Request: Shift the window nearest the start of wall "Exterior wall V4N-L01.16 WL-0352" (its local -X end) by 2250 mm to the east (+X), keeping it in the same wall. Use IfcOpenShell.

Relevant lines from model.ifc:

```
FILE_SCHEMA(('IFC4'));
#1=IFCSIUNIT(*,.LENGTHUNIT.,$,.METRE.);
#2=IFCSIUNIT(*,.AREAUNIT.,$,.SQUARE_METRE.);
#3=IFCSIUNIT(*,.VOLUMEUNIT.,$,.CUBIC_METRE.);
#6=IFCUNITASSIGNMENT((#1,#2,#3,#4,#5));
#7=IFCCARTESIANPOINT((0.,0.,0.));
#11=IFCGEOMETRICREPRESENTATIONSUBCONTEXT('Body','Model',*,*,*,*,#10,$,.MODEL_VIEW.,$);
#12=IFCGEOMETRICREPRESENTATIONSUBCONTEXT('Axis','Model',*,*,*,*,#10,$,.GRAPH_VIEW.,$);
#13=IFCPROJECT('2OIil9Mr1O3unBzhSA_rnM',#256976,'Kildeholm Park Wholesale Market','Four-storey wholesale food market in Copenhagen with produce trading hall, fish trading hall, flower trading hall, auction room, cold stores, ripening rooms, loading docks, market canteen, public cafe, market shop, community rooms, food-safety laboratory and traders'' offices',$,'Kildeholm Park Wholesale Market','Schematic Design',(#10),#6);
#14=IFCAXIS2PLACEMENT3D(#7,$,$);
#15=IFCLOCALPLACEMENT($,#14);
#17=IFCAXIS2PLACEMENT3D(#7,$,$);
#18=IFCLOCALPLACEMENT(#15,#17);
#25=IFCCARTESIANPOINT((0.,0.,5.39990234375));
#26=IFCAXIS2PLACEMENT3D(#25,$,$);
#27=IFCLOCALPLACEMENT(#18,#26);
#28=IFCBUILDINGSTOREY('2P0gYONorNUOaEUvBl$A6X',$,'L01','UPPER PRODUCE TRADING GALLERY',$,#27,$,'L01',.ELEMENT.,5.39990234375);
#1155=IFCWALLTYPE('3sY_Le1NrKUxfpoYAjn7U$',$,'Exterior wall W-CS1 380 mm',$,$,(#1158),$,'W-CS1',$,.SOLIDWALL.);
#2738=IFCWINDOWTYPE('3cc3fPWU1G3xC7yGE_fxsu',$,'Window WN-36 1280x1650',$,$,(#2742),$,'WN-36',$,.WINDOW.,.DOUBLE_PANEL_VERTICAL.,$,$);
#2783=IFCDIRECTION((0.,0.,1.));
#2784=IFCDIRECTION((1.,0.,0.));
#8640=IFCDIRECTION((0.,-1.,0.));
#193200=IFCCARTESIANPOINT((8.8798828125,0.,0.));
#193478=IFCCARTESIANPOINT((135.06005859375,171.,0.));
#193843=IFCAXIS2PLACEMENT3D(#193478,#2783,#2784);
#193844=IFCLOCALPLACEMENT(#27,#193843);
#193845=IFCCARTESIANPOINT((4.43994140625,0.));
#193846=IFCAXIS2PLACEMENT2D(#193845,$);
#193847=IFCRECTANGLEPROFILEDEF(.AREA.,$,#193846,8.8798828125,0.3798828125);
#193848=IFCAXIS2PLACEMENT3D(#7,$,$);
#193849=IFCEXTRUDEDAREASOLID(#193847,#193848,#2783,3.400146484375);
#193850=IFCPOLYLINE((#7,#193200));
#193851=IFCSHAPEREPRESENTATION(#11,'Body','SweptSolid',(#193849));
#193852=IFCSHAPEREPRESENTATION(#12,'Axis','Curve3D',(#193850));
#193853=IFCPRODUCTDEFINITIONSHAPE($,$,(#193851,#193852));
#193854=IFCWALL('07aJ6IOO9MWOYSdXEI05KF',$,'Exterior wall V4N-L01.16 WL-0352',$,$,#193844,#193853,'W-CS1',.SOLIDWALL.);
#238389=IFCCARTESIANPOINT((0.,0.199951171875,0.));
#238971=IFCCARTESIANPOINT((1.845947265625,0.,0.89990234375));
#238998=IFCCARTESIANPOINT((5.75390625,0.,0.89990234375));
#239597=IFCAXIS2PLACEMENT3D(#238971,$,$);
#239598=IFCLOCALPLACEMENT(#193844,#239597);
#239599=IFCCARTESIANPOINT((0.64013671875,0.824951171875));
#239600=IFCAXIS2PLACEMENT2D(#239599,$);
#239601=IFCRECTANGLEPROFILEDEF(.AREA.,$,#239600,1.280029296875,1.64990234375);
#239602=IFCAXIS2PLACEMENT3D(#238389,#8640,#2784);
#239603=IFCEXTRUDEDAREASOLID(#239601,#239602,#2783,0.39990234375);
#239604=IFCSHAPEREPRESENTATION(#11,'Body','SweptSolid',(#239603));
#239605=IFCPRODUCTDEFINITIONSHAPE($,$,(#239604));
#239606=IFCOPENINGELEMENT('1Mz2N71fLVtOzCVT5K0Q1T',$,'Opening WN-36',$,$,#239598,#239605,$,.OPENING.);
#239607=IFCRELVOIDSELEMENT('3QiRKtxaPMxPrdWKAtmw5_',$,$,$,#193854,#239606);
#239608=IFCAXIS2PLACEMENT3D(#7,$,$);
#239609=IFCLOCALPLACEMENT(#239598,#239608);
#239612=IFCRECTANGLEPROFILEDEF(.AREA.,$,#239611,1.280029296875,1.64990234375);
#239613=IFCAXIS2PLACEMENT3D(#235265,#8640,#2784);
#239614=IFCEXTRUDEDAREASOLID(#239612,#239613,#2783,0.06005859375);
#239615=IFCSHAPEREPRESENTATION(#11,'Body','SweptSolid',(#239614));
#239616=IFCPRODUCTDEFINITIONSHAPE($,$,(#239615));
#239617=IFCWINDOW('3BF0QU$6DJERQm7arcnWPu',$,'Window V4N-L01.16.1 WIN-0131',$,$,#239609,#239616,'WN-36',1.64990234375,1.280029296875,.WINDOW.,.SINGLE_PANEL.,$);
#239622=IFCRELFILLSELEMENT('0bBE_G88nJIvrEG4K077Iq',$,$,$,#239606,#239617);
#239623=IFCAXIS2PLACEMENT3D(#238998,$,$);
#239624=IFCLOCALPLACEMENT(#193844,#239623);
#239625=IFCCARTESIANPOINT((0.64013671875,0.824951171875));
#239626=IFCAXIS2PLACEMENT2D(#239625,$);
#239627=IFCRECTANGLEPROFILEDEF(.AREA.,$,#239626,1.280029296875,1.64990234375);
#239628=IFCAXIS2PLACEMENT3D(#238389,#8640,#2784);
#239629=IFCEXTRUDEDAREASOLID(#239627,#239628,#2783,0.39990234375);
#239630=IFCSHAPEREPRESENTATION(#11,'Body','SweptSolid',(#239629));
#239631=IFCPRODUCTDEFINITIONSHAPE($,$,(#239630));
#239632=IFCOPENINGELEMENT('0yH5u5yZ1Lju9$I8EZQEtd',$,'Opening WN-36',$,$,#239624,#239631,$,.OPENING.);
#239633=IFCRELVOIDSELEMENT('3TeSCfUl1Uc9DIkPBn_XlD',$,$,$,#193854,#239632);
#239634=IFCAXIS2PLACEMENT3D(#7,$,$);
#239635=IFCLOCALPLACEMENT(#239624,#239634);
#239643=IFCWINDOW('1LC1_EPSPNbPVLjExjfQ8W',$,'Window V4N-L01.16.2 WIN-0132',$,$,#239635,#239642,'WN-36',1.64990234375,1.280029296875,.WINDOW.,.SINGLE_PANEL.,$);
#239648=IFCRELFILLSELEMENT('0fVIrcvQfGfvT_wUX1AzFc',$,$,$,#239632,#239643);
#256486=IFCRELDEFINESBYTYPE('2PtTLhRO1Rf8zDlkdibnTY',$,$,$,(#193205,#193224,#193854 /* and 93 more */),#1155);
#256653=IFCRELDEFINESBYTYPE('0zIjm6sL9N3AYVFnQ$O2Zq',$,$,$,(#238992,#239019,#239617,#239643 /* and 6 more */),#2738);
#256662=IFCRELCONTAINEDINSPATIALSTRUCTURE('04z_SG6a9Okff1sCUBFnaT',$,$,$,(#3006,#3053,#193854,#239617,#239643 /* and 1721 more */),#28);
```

```python
import ifcopenshell
import ifcopenshell.api.geometry
import ifcopenshell.util.placement

model = ifcopenshell.open("model.ifc")

window = model.by_id(239617)
opening = window.FillsVoids[0].RelatingOpeningElement
wall = opening.VoidsElements[0].RelatingBuildingElement

wall_matrix = ifcopenshell.util.placement.get_local_placement(wall.ObjectPlacement)
shift = wall_matrix[:3, 0] * 2.25
before = ifcopenshell.util.placement.get_local_placement(window.ObjectPlacement)[:3, 3].copy()

# The window is placed relative to its opening, so it follows when the opening moves.
matrix = ifcopenshell.util.placement.get_local_placement(opening.ObjectPlacement)
matrix[:3, 3] += shift
ifcopenshell.api.geometry.edit_object_placement(
    model, product=opening, matrix=matrix, is_si=False, should_transform_children=True
)

after = ifcopenshell.util.placement.get_local_placement(window.ObjectPlacement)[:3, 3]
print("window moved by", (after - before).round(3) + 0.0)

model.write("model_updated.ifc")
```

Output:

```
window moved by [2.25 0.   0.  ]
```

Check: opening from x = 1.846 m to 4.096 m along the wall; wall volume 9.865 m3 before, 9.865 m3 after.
